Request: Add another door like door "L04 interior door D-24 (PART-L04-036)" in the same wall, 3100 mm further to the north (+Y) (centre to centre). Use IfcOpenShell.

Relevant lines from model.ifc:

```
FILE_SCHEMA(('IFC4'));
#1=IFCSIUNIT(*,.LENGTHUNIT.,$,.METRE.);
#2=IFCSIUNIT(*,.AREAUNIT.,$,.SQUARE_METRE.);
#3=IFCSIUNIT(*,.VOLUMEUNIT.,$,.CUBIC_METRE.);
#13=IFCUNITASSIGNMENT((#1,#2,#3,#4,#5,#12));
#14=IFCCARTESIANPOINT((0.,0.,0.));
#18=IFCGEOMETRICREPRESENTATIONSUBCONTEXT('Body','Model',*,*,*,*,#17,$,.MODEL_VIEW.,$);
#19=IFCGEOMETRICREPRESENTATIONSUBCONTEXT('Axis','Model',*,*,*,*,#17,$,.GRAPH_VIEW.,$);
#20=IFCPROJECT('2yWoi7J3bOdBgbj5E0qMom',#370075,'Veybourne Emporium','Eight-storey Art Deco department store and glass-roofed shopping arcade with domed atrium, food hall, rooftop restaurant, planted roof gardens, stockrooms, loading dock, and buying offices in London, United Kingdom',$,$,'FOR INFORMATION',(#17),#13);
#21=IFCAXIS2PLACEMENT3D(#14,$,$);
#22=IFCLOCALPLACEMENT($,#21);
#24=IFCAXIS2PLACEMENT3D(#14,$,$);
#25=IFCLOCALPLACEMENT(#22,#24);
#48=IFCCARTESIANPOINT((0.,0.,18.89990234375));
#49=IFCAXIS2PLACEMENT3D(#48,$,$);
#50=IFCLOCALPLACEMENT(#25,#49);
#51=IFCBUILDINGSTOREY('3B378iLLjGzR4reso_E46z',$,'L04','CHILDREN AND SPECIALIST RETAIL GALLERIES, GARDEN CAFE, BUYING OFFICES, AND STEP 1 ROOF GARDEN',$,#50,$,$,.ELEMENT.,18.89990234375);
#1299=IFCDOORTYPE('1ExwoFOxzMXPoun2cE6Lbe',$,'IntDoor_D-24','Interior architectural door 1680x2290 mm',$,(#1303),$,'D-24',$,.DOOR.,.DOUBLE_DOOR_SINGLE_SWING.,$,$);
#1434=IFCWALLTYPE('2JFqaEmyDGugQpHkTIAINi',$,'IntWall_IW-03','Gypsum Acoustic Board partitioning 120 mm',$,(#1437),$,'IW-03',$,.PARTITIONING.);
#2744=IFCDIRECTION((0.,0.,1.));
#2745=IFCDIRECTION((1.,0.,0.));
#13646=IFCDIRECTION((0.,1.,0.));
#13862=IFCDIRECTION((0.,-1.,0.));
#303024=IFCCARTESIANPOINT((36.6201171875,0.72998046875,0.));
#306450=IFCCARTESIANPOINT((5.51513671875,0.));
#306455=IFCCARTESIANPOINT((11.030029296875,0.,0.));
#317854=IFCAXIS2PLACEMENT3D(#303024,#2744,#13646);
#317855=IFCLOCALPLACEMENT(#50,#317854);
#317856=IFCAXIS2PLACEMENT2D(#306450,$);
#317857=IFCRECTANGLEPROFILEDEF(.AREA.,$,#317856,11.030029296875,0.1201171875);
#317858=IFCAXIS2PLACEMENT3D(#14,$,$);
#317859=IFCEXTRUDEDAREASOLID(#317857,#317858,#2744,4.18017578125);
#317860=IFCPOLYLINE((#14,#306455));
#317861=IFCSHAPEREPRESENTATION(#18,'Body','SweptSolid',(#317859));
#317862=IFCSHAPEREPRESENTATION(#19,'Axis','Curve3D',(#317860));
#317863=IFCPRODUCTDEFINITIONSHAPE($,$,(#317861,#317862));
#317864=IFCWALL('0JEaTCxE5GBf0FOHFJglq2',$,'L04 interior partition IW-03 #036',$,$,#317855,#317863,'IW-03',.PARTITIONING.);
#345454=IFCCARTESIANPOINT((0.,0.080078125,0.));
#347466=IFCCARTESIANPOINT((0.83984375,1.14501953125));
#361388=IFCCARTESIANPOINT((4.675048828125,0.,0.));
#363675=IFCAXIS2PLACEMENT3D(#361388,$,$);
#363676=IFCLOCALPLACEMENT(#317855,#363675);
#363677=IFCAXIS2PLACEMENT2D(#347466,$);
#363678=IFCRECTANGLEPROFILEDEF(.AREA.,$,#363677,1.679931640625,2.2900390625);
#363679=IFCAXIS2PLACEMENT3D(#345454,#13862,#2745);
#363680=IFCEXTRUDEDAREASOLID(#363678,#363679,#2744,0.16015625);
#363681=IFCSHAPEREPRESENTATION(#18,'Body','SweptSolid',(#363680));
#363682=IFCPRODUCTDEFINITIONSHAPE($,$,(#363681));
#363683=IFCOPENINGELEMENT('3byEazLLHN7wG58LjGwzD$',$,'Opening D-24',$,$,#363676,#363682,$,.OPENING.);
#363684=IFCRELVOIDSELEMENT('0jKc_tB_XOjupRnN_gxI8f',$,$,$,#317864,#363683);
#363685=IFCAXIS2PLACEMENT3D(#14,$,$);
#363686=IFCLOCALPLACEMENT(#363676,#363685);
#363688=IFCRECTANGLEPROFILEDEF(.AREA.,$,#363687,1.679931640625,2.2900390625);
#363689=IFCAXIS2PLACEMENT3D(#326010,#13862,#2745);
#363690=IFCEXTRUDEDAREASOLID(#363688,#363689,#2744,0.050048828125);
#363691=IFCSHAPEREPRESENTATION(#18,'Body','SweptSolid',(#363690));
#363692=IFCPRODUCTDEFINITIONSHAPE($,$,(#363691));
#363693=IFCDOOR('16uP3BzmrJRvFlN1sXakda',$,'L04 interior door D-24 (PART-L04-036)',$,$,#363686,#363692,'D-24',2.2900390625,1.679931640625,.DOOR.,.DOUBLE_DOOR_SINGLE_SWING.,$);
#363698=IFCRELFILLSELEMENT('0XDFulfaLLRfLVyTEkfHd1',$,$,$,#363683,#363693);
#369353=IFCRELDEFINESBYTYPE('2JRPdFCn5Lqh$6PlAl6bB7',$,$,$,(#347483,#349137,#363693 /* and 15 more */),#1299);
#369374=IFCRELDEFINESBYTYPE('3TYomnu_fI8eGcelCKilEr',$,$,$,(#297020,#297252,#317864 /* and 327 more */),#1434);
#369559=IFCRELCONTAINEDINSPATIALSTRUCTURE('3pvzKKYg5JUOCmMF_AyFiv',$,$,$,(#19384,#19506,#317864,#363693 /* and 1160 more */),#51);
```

```python
import ifcopenshell
import ifcopenshell.api.feature
import ifcopenshell.api.geometry
import ifcopenshell.api.root
import ifcopenshell.geom
import ifcopenshell.util.element
import ifcopenshell.util.placement
import ifcopenshell.util.shape
import ifcopenshell.util.unit

model = ifcopenshell.open("model.ifc")
unit_scale = ifcopenshell.util.unit.calculate_unit_scale(model)
settings = ifcopenshell.geom.settings()


def volume(element):
    """Net volume in cubic metres, openings subtracted."""
    shape = ifcopenshell.geom.create_shape(settings, element)
    return ifcopenshell.util.shape.get_volume(shape.geometry)


door = model.by_id(363693)
opening = door.FillsVoids[0].RelatingOpeningElement
wall = opening.VoidsElements[0].RelatingBuildingElement
before = volume(wall)
shift = ifcopenshell.util.placement.get_local_placement(wall.ObjectPlacement)[:3, 0] * 3.1 / unit_scale

# copy_class copies the void relationship, type, container and properties, but no geometry.
new_opening = ifcopenshell.api.root.copy_class(model, product=opening)
new_opening.Representation = ifcopenshell.util.element.copy_deep(
    model, opening.Representation, exclude=["IfcGeometricRepresentationContext", "IfcRepresentationMap"]
)
new_door = ifcopenshell.api.root.copy_class(model, product=door)
new_door.Representation = ifcopenshell.util.element.copy_deep(
    model, door.Representation, exclude=["IfcGeometricRepresentationContext", "IfcRepresentationMap"]
)
new_door.Tag = None
ifcopenshell.api.feature.add_filling(model, opening=new_opening, element=new_door)

for old, new in ((opening, new_opening), (door, new_door)):
    matrix = ifcopenshell.util.placement.get_local_placement(old.ObjectPlacement)
    matrix[:3, 3] += shift
    ifcopenshell.api.geometry.edit_object_placement(model, product=new, matrix=matrix, is_si=False)

after = volume(wall)

print(f"wall volume {before:.3f} -> {after:.3f} m3")

model.write("model_edited.ifc")
```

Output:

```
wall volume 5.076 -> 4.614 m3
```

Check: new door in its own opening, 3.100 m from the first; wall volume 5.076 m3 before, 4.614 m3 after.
